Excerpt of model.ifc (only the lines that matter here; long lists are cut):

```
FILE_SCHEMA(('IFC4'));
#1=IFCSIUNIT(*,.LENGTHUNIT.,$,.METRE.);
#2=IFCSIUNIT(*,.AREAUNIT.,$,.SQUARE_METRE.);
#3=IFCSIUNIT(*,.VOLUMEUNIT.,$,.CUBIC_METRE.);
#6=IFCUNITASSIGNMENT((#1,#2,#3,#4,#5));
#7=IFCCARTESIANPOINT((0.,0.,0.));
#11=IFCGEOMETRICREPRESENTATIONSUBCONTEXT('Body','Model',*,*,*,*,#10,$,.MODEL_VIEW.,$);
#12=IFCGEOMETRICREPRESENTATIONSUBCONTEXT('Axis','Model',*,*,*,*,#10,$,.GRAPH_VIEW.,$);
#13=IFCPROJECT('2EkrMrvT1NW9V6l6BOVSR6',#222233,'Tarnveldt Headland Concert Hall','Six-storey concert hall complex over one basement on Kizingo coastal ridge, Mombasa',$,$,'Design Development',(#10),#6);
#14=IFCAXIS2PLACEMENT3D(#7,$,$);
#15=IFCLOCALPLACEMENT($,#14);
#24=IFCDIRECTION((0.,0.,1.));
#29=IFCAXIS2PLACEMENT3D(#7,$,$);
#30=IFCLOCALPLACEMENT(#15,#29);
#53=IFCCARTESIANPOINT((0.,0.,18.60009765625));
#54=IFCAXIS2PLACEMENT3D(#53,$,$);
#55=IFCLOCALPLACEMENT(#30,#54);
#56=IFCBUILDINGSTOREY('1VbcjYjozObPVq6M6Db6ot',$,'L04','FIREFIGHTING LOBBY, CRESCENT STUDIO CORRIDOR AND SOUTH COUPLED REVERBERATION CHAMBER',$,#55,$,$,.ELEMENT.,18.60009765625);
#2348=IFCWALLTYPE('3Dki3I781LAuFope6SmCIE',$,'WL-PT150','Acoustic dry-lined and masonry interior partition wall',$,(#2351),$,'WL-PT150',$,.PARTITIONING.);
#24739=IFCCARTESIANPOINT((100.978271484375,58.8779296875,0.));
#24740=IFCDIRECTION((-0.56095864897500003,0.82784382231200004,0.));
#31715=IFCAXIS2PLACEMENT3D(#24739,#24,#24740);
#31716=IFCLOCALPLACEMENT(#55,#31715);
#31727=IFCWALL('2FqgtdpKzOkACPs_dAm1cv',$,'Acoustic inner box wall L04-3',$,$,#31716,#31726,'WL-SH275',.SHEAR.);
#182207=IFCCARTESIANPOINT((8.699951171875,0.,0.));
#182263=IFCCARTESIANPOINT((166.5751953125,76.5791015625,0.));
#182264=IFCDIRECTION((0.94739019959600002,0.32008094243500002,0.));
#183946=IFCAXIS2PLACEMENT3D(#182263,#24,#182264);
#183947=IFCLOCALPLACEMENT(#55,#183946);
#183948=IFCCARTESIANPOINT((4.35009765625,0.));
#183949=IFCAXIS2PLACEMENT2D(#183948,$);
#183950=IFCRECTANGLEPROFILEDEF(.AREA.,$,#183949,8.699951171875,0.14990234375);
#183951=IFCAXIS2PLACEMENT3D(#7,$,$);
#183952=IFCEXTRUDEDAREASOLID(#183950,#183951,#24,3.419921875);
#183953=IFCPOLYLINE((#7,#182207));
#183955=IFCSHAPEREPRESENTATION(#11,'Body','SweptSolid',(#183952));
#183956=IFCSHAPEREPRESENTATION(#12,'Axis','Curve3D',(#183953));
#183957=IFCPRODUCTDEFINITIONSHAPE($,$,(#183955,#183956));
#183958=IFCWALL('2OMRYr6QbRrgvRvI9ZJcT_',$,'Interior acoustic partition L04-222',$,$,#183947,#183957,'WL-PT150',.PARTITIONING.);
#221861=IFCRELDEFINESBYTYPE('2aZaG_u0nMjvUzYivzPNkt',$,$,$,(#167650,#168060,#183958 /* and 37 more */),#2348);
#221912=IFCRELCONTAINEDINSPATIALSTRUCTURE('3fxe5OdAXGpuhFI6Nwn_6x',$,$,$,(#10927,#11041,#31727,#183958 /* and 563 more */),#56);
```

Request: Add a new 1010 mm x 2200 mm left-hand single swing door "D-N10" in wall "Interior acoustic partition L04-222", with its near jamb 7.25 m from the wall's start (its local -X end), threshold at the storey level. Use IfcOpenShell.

```python
import numpy as np
import ifcopenshell
import ifcopenshell.api.feature
import ifcopenshell.api.geometry
import ifcopenshell.api.root
import ifcopenshell.api.spatial
import ifcopenshell.geom
import ifcopenshell.util.element
import ifcopenshell.util.placement
import ifcopenshell.util.representation
import ifcopenshell.util.shape
import ifcopenshell.util.unit

model = ifcopenshell.open("model.ifc")
unit_scale = ifcopenshell.util.unit.calculate_unit_scale(model)
settings = ifcopenshell.geom.settings()


def volume(element):
    """Net volume in cubic metres, openings subtracted."""
    shape = ifcopenshell.geom.create_shape(settings, element)
    return ifcopenshell.util.shape.get_volume(shape.geometry)


wall = model.by_guid("2OMRYr6QbRrgvRvI9ZJcT_")
storey = ifcopenshell.util.element.get_container(wall, ifc_class="IfcBuildingStorey")
context = ifcopenshell.util.representation.get_context(model, "Model", "Body", "MODEL_VIEW")
before = volume(wall)

width, height, from_end, sill = 1.01, 2.2, 7.25, 0.0  # metres

# The wall runs along its own X axis, and the end named is its -X end.
wall_shape = ifcopenshell.geom.create_shape(settings, wall)
x, y, z = ifcopenshell.util.shape.get_vertices(wall_shape.geometry).T
start = x.min() + from_end
face, thickness = float(y.min()), float(y.max() - y.min())
wall_matrix = ifcopenshell.util.placement.get_local_placement(wall.ObjectPlacement)
level = ifcopenshell.util.placement.get_local_placement(storey.ObjectPlacement)[2, 3]


def in_wall(x, y):
    """Placement at x, y metres in the wall's axes, at sill height."""
    matrix = wall_matrix.copy()
    matrix[:, 3] = wall_matrix @ np.array([x / unit_scale, y / unit_scale, 0.0, 1.0])
    matrix[2, 3] = level + sill / unit_scale
    return matrix


# Opening: a box that overshoots both wall faces by 50 mm.
opening = ifcopenshell.api.root.create_entity(model, ifc_class="IfcOpeningElement", predefined_type="OPENING")
box = ifcopenshell.api.geometry.add_wall_representation(
    model, context=context, length=width, height=height, thickness=thickness + 0.1
)
ifcopenshell.api.geometry.assign_representation(model, product=opening, representation=box)
ifcopenshell.api.geometry.edit_object_placement(model, product=opening, matrix=in_wall(start, face - 0.05), is_si=False)
ifcopenshell.api.feature.add_feature(model, feature=opening, element=wall)

door = ifcopenshell.api.root.create_entity(model, ifc_class="IfcDoor", name="D-N10", predefined_type="DOOR")
door.OverallWidth, door.OverallHeight = width / unit_scale, height / unit_scale
door.OperationType = "SINGLE_SWING_LEFT"
body = ifcopenshell.api.geometry.add_door_representation(
    model,
    context=context,
    overall_width=door.OverallWidth,
    overall_height=door.OverallHeight,
    operation_type="SINGLE_SWING_LEFT",
    lining_properties={"LiningDepth": thickness / unit_scale, "ThresholdDepth": thickness / unit_scale},
)
ifcopenshell.api.geometry.assign_representation(model, product=door, representation=body)
ifcopenshell.api.spatial.assign_container(model, products=[door], relating_structure=storey)
ifcopenshell.api.feature.add_filling(model, opening=opening, element=door)

# The lining spans the wall, so the door starts at the wall face.
ifcopenshell.api.geometry.edit_object_placement(model, product=door, matrix=in_wall(start, face), is_si=False)

after = volume(wall)

print(f"wall volume {before:.3f} -> {after:.3f} m3")

model.write("model-out.ifc")
```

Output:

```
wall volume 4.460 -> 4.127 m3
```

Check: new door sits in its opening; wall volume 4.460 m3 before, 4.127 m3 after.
